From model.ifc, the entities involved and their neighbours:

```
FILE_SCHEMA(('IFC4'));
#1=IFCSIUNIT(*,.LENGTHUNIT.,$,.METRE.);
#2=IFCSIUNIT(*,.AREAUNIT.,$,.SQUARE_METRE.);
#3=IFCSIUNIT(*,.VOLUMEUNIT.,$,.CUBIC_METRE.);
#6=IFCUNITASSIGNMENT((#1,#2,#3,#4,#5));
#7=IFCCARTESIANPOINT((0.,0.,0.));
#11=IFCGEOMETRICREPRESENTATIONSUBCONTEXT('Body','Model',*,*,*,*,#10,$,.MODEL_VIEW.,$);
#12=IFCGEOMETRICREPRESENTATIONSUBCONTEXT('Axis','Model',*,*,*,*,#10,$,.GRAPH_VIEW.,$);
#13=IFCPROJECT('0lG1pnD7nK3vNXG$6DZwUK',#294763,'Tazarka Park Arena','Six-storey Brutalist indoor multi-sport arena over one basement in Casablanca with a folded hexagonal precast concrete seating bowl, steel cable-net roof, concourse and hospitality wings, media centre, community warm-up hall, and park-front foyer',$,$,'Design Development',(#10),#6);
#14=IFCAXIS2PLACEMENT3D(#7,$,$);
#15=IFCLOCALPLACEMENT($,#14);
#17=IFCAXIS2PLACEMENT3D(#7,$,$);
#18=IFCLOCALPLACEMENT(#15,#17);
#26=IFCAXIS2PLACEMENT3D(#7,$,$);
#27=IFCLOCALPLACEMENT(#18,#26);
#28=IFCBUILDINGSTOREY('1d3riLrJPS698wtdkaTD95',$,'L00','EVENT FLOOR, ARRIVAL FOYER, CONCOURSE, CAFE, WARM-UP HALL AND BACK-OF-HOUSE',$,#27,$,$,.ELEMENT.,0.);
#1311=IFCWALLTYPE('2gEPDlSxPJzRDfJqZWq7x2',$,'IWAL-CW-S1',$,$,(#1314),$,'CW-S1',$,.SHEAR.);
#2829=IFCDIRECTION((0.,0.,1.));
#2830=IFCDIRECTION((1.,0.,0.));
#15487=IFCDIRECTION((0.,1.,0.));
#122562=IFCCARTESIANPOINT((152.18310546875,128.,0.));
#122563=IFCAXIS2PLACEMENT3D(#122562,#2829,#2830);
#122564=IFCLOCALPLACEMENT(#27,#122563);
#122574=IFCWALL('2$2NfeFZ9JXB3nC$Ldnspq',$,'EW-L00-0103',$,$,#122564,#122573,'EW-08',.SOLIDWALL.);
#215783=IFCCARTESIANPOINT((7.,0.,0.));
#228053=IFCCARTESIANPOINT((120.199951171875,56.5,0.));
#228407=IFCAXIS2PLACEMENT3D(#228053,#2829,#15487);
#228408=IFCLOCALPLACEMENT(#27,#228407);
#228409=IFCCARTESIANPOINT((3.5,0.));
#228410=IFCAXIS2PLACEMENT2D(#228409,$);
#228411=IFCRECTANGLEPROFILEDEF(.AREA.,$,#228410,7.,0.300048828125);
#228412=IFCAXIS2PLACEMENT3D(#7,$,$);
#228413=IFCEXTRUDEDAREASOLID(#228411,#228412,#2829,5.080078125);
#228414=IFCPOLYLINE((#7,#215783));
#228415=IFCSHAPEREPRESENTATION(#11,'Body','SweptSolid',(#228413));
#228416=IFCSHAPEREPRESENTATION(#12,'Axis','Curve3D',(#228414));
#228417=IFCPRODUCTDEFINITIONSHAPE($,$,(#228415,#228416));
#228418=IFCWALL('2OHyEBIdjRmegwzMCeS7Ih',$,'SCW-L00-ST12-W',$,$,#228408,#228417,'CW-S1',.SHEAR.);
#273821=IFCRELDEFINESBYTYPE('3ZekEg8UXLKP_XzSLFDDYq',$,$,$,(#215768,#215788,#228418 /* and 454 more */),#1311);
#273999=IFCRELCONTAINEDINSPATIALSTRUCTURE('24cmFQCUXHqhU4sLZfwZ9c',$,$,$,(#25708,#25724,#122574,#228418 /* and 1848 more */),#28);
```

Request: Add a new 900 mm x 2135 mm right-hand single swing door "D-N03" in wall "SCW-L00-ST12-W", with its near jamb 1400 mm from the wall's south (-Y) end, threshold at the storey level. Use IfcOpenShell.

```python
import numpy as np
import ifcopenshell
import ifcopenshell.api.feature
import ifcopenshell.api.geometry
import ifcopenshell.api.root
import ifcopenshell.api.spatial
import ifcopenshell.geom
import ifcopenshell.util.element
import ifcopenshell.util.placement
import ifcopenshell.util.representation
import ifcopenshell.util.shape
import ifcopenshell.util.unit

model = ifcopenshell.open("model.ifc")
unit_scale = ifcopenshell.util.unit.calculate_unit_scale(model)
settings = ifcopenshell.geom.settings()


def volume(element):
    """Net volume in cubic metres, openings subtracted."""
    shape = ifcopenshell.geom.create_shape(settings, element)
    return ifcopenshell.util.shape.get_volume(shape.geometry)


wall = model.by_guid("2OHyEBIdjRmegwzMCeS7Ih")
storey = ifcopenshell.util.element.get_container(wall, ifc_class="IfcBuildingStorey")
context = ifcopenshell.util.representation.get_context(model, "Model", "Body", "MODEL_VIEW")
before = volume(wall)

width, height, from_end, sill = 0.9, 2.135, 1.4, 0.0  # metres

# The wall runs along its own X axis, and the end named is its -X end.
wall_shape = ifcopenshell.geom.create_shape(settings, wall)
x, y, z = ifcopenshell.util.shape.get_vertices(wall_shape.geometry).T
start = x.min() + from_end
face, thickness = float(y.min()), float(y.max() - y.min())
wall_matrix = ifcopenshell.util.placement.get_local_placement(wall.ObjectPlacement)
level = ifcopenshell.util.placement.get_local_placement(storey.ObjectPlacement)[2, 3]


def in_wall(x, y):
    """Placement at x, y metres in the wall's axes, at sill height."""
    matrix = wall_matrix.copy()
    matrix[:, 3] = wall_matrix @ np.array([x / unit_scale, y / unit_scale, 0.0, 1.0])
    matrix[2, 3] = level + sill / unit_scale
    return matrix


# Opening: a box that overshoots both wall faces by 50 mm.
opening = ifcopenshell.api.root.create_entity(model, ifc_class="IfcOpeningElement", predefined_type="OPENING")
box = ifcopenshell.api.geometry.add_wall_representation(
    model, context=context, length=width, height=height, thickness=thickness + 0.1
)
ifcopenshell.api.geometry.assign_representation(model, product=opening, representation=box)
ifcopenshell.api.geometry.edit_object_placement(model, product=opening, matrix=in_wall(start, face - 0.05), is_si=False)
ifcopenshell.api.feature.add_feature(model, feature=opening, element=wall)

door = ifcopenshell.api.root.create_entity(model, ifc_class="IfcDoor", name="D-N03", predefined_type="DOOR")
door.OverallWidth, door.OverallHeight = width / unit_scale, height / unit_scale
door.OperationType = "SINGLE_SWING_RIGHT"
body = ifcopenshell.api.geometry.add_door_representation(
    model,
    context=context,
    overall_width=door.OverallWidth,
    overall_height=door.OverallHeight,
    operation_type="SINGLE_SWING_RIGHT",
    lining_properties={"LiningDepth": thickness / unit_scale, "ThresholdDepth": thickness / unit_scale},
)
ifcopenshell.api.geometry.assign_representation(model, product=door, representation=body)
ifcopenshell.api.spatial.assign_container(model, products=[door], relating_structure=storey)
ifcopenshell.api.feature.add_filling(model, opening=opening, element=door)

# The lining spans the wall, so the door starts at the wall face.
ifcopenshell.api.geometry.edit_object_placement(model, product=door, matrix=in_wall(start, face), is_si=False)

after = volume(wall)

print(f"wall volume {before:.3f} -> {after:.3f} m3")

model.write("model_v2.ifc")
```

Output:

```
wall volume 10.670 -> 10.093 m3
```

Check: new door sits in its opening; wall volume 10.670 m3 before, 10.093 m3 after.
